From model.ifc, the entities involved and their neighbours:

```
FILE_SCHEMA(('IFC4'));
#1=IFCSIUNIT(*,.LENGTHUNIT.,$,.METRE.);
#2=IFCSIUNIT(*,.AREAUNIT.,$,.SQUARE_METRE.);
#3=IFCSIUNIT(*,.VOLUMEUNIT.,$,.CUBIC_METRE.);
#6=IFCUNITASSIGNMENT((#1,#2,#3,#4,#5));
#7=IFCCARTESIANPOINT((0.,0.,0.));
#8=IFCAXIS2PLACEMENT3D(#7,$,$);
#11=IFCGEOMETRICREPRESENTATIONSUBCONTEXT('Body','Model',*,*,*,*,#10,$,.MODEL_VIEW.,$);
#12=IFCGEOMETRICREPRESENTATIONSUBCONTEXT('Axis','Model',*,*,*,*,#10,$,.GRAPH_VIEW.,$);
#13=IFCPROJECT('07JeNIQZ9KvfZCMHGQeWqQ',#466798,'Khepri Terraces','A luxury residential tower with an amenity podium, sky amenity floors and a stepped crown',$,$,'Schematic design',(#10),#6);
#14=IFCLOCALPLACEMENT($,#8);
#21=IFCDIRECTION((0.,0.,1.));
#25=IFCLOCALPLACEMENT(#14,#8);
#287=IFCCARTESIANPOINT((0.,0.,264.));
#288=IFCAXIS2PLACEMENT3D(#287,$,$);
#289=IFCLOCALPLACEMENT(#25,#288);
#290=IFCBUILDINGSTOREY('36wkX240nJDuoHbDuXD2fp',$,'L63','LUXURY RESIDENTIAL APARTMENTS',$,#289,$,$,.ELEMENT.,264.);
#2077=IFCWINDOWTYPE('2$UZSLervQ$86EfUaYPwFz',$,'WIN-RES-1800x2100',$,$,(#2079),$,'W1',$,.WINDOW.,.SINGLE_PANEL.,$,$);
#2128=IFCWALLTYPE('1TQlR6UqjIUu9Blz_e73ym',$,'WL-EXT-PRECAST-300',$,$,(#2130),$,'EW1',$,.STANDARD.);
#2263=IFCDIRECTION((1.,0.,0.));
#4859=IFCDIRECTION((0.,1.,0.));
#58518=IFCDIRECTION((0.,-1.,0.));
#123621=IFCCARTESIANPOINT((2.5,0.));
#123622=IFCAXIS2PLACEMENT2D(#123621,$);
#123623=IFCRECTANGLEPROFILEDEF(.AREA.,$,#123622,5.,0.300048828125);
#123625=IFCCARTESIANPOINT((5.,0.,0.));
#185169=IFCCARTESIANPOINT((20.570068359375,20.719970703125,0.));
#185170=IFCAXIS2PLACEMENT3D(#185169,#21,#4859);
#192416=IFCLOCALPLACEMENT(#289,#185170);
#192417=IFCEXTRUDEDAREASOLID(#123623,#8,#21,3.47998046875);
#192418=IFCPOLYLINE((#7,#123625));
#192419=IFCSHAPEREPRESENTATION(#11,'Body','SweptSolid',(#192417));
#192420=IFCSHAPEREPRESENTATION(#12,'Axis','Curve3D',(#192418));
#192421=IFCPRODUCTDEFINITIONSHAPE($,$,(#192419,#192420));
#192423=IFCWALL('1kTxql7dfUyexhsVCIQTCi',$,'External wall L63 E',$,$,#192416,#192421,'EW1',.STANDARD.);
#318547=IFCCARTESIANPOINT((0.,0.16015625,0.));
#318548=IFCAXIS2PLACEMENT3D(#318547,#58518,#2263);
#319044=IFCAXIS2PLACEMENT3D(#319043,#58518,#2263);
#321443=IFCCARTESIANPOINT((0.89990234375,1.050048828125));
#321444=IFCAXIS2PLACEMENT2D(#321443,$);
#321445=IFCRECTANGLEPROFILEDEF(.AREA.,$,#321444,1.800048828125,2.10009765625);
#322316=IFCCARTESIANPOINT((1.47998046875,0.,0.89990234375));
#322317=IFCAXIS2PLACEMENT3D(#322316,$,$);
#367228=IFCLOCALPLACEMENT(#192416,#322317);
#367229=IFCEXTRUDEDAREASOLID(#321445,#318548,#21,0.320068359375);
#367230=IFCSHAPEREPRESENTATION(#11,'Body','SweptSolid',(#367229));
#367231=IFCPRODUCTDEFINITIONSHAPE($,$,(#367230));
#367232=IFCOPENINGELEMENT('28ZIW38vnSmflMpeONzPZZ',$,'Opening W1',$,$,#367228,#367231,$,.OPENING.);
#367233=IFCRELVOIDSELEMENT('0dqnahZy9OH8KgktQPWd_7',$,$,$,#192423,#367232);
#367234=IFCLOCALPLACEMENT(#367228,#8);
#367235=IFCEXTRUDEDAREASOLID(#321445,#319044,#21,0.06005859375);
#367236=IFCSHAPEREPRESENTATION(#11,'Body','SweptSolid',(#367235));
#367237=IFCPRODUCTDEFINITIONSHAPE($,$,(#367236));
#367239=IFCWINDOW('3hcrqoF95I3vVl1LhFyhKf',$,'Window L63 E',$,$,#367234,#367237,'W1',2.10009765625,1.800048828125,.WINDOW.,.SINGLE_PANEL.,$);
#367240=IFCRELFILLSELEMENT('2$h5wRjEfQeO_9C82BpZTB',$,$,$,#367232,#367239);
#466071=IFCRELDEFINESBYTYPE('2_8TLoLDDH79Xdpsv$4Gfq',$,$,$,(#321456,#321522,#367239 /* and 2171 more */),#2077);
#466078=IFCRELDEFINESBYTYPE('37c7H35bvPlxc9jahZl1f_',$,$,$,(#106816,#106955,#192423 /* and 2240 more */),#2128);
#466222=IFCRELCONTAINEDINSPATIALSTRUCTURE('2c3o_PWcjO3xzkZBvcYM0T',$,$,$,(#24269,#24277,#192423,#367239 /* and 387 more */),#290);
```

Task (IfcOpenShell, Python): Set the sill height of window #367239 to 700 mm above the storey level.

```python
import numpy as np
import ifcopenshell
import ifcopenshell.api.geometry
import ifcopenshell.geom
import ifcopenshell.util.element
import ifcopenshell.util.placement
import ifcopenshell.util.shape
import ifcopenshell.util.unit

model = ifcopenshell.open("model.ifc")
unit_scale = ifcopenshell.util.unit.calculate_unit_scale(model)

window = model.by_guid("3hcrqoF95I3vVl1LhFyhKf")
opening = window.FillsVoids[0].RelatingOpeningElement
storey = ifcopenshell.util.element.get_container(window, ifc_class="IfcBuildingStorey")
level = ifcopenshell.util.placement.get_local_placement(storey.ObjectPlacement)[2, 3]

# The opening's origin need not be at the sill, so measure its lowest point.
shape = ifcopenshell.geom.create_shape(ifcopenshell.geom.settings(), opening)
bottom = ifcopenshell.util.shape.get_shape_bottom_elevation(shape, shape.geometry) / unit_scale
dz = level + 0.7 / unit_scale - bottom

shift = np.array([0.0, 0.0, dz])
# The window is placed relative to its opening, so it follows when the opening moves.
matrix = ifcopenshell.util.placement.get_local_placement(opening.ObjectPlacement)
matrix[:3, 3] += shift
ifcopenshell.api.geometry.edit_object_placement(
    model, product=opening, matrix=matrix, is_si=False, should_transform_children=True
)

print(f"moved by {dz * unit_scale:+.3f} m")

model.write("model-out.ifc")
```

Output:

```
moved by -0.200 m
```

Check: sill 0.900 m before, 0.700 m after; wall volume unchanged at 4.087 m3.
